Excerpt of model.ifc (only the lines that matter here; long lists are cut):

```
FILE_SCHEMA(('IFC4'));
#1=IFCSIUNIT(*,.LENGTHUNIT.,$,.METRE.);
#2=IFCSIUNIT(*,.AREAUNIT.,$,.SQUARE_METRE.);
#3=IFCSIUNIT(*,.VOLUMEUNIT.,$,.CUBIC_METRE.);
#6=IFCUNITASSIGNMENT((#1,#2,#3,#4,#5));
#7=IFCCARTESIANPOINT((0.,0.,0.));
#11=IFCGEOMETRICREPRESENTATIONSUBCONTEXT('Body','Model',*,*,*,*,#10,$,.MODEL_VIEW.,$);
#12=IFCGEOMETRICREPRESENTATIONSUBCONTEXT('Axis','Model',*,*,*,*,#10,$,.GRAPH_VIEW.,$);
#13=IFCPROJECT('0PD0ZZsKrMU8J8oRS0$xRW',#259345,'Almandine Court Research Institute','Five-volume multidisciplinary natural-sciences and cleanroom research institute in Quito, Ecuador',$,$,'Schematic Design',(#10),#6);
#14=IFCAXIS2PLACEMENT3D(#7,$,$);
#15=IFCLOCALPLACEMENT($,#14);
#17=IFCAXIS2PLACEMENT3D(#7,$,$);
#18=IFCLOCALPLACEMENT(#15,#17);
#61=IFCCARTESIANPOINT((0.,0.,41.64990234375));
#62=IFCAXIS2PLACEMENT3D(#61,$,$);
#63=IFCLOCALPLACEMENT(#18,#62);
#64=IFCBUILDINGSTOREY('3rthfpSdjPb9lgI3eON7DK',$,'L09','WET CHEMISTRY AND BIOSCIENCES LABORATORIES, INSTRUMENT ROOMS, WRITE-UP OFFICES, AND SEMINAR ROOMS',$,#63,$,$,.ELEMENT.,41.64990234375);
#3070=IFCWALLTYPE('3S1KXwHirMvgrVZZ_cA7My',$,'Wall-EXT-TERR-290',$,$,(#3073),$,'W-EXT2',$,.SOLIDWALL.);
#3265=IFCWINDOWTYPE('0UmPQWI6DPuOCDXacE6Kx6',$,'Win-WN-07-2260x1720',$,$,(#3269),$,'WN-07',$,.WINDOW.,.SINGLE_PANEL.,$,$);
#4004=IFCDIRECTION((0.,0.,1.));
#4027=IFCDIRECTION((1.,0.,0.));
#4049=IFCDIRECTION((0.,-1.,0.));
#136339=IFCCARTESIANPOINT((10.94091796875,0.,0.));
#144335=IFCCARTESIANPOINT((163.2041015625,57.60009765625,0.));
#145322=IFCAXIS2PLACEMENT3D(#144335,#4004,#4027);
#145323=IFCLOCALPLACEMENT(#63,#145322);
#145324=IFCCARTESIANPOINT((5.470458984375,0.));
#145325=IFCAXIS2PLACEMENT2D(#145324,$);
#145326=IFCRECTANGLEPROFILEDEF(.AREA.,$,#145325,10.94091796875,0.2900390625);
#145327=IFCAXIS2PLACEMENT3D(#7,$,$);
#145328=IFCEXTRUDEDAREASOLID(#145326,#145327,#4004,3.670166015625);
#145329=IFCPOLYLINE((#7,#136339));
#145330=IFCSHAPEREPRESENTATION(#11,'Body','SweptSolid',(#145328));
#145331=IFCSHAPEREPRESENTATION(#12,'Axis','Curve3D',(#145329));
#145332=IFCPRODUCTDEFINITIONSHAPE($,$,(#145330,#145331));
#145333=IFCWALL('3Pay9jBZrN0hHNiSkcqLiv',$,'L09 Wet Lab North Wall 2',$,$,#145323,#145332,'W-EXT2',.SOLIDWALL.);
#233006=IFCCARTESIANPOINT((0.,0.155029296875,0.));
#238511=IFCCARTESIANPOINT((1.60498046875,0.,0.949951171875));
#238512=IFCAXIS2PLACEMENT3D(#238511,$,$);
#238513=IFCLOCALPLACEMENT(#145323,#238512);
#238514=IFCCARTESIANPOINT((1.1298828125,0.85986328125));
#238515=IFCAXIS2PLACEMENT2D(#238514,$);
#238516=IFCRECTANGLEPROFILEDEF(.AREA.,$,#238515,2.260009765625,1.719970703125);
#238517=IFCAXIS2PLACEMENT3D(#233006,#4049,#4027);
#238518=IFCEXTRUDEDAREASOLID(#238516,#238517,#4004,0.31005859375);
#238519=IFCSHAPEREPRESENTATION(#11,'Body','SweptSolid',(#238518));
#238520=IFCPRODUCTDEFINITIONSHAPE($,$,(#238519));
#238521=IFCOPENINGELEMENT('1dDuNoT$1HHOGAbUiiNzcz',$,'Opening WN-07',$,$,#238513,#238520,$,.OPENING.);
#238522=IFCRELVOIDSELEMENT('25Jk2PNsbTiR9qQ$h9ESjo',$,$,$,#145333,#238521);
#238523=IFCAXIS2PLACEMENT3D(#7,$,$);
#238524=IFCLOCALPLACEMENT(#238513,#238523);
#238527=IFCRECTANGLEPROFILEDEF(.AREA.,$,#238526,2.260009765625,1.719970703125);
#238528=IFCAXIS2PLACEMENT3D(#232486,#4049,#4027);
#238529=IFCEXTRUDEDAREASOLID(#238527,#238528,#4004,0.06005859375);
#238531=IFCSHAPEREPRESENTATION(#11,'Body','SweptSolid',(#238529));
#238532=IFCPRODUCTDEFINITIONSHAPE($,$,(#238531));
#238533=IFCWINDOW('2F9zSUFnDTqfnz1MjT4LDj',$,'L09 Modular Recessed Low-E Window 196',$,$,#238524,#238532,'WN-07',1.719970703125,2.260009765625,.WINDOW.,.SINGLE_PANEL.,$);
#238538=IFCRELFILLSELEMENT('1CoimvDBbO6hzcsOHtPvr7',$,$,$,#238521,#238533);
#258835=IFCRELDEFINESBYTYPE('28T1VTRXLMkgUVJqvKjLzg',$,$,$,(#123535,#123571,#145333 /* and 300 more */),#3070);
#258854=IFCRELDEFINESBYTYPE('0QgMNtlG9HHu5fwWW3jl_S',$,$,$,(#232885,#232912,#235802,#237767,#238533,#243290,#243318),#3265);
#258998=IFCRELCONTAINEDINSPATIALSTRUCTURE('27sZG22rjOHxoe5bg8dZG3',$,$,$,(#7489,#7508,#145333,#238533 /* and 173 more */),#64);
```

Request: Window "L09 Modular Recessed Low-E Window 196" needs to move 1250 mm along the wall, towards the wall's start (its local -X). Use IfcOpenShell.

```python
import ifcopenshell
import ifcopenshell.api.geometry
import ifcopenshell.util.placement

model = ifcopenshell.open("model.ifc")

window = model.by_id(238533)
opening = window.FillsVoids[0].RelatingOpeningElement
wall = opening.VoidsElements[0].RelatingBuildingElement

wall_matrix = ifcopenshell.util.placement.get_local_placement(wall.ObjectPlacement)
shift = wall_matrix[:3, 0] * -1.25
before = ifcopenshell.util.placement.get_local_placement(window.ObjectPlacement)[:3, 3].copy()

# The window is placed relative to its opening, so it follows when the opening moves.
matrix = ifcopenshell.util.placement.get_local_placement(opening.ObjectPlacement)
matrix[:3, 3] += shift
ifcopenshell.api.geometry.edit_object_placement(
    model, product=opening, matrix=matrix, is_si=False, should_transform_children=True
)

after = ifcopenshell.util.placement.get_local_placement(window.ObjectPlacement)[:3, 3]
print("window moved by", (after - before).round(3) + 0.0)

model.write("model_v2.ifc")
```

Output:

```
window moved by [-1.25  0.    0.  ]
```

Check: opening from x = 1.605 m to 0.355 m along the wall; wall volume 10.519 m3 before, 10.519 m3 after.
